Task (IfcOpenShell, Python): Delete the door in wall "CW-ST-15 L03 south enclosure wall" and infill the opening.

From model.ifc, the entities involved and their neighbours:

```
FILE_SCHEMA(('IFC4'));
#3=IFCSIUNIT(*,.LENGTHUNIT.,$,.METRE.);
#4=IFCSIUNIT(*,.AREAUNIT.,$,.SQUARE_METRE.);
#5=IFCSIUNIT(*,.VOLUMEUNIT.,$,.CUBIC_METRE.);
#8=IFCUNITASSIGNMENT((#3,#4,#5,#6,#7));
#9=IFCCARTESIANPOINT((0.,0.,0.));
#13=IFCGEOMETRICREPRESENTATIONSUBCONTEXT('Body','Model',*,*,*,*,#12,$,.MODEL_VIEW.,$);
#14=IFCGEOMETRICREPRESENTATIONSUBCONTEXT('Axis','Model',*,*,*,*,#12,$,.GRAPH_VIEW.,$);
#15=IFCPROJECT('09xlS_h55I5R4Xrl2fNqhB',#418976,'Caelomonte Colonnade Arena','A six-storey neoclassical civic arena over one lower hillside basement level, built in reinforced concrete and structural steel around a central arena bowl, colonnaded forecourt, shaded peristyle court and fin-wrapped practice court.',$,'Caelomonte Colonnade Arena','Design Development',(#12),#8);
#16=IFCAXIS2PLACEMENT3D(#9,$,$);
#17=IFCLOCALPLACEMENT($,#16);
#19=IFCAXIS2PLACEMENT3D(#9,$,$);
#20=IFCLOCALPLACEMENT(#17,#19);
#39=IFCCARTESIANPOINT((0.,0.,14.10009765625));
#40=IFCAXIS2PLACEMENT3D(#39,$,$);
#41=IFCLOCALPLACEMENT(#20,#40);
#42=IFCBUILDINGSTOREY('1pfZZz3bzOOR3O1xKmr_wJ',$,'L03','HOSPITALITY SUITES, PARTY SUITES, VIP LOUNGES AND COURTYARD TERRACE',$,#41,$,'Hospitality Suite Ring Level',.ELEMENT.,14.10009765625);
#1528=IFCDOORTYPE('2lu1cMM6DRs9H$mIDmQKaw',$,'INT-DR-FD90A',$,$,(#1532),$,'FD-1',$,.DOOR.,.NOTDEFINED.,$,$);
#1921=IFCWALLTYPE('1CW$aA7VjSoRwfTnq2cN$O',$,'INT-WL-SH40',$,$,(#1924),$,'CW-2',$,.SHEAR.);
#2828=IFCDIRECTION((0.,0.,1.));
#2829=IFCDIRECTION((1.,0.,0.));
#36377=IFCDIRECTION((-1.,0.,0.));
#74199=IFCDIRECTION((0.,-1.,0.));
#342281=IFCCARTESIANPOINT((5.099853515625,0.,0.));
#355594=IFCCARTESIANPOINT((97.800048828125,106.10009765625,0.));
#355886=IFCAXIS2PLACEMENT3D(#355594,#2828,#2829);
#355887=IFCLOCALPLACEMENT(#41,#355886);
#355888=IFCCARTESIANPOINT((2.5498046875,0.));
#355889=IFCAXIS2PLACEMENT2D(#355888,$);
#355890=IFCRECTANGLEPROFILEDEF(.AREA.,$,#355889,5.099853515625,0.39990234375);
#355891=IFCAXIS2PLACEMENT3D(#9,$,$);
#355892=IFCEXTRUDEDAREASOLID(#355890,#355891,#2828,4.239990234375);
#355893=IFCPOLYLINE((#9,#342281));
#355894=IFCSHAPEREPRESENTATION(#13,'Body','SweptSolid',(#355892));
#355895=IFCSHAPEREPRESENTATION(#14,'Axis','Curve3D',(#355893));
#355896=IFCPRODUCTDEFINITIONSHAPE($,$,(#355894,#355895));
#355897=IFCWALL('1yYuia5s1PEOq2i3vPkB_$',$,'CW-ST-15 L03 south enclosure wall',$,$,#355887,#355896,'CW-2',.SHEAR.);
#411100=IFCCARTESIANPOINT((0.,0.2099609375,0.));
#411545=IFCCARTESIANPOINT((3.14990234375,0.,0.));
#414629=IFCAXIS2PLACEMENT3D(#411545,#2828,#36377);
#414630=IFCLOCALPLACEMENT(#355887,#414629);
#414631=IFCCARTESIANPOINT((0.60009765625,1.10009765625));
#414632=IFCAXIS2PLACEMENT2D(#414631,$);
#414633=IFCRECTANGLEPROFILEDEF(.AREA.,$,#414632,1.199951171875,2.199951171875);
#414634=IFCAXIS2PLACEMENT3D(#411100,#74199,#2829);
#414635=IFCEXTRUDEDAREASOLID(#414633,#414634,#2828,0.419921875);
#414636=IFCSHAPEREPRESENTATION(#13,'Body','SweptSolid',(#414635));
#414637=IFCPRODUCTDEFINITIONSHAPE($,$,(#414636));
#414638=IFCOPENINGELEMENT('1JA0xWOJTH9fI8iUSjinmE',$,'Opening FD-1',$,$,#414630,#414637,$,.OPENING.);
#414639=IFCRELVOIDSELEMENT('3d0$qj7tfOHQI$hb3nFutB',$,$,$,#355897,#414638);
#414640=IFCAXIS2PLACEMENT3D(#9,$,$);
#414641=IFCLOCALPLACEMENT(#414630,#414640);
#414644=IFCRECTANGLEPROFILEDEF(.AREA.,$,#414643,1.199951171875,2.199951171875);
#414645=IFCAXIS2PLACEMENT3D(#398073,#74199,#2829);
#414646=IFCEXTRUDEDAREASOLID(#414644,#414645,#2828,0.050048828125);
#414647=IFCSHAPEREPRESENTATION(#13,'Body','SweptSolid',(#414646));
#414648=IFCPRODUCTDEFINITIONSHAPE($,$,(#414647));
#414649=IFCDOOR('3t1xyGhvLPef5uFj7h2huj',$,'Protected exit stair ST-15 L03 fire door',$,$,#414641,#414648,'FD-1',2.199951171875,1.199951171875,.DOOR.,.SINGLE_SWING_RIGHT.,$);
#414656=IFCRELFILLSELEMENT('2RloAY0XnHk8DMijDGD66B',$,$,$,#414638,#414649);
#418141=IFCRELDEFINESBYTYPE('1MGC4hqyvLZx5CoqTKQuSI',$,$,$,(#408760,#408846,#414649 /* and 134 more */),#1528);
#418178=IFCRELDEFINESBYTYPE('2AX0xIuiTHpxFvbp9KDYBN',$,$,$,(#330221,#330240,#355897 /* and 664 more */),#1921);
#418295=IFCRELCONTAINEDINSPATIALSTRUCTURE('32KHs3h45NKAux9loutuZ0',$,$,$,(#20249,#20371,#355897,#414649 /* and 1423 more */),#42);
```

```python
import ifcopenshell
import ifcopenshell.api.feature
import ifcopenshell.api.root
import ifcopenshell.geom
import ifcopenshell.util.shape

model = ifcopenshell.open("model.ifc")
settings = ifcopenshell.geom.settings()


def volume(element):
    """Net volume in cubic metres, openings subtracted."""
    shape = ifcopenshell.geom.create_shape(settings, element)
    return ifcopenshell.util.shape.get_volume(shape.geometry)


door = model.by_guid("3t1xyGhvLPef5uFj7h2huj")
opening = door.FillsVoids[0].RelatingOpeningElement
wall = opening.VoidsElements[0].RelatingBuildingElement
before = volume(wall)

ifcopenshell.api.root.remove_product(model, product=door)
ifcopenshell.api.feature.remove_feature(model, feature=opening)

after = volume(wall)

print(f"wall volume {before:.3f} -> {after:.3f} m3")

model.write("model_updated.ifc")
```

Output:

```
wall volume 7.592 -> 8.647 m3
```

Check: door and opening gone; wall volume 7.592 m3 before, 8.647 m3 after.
